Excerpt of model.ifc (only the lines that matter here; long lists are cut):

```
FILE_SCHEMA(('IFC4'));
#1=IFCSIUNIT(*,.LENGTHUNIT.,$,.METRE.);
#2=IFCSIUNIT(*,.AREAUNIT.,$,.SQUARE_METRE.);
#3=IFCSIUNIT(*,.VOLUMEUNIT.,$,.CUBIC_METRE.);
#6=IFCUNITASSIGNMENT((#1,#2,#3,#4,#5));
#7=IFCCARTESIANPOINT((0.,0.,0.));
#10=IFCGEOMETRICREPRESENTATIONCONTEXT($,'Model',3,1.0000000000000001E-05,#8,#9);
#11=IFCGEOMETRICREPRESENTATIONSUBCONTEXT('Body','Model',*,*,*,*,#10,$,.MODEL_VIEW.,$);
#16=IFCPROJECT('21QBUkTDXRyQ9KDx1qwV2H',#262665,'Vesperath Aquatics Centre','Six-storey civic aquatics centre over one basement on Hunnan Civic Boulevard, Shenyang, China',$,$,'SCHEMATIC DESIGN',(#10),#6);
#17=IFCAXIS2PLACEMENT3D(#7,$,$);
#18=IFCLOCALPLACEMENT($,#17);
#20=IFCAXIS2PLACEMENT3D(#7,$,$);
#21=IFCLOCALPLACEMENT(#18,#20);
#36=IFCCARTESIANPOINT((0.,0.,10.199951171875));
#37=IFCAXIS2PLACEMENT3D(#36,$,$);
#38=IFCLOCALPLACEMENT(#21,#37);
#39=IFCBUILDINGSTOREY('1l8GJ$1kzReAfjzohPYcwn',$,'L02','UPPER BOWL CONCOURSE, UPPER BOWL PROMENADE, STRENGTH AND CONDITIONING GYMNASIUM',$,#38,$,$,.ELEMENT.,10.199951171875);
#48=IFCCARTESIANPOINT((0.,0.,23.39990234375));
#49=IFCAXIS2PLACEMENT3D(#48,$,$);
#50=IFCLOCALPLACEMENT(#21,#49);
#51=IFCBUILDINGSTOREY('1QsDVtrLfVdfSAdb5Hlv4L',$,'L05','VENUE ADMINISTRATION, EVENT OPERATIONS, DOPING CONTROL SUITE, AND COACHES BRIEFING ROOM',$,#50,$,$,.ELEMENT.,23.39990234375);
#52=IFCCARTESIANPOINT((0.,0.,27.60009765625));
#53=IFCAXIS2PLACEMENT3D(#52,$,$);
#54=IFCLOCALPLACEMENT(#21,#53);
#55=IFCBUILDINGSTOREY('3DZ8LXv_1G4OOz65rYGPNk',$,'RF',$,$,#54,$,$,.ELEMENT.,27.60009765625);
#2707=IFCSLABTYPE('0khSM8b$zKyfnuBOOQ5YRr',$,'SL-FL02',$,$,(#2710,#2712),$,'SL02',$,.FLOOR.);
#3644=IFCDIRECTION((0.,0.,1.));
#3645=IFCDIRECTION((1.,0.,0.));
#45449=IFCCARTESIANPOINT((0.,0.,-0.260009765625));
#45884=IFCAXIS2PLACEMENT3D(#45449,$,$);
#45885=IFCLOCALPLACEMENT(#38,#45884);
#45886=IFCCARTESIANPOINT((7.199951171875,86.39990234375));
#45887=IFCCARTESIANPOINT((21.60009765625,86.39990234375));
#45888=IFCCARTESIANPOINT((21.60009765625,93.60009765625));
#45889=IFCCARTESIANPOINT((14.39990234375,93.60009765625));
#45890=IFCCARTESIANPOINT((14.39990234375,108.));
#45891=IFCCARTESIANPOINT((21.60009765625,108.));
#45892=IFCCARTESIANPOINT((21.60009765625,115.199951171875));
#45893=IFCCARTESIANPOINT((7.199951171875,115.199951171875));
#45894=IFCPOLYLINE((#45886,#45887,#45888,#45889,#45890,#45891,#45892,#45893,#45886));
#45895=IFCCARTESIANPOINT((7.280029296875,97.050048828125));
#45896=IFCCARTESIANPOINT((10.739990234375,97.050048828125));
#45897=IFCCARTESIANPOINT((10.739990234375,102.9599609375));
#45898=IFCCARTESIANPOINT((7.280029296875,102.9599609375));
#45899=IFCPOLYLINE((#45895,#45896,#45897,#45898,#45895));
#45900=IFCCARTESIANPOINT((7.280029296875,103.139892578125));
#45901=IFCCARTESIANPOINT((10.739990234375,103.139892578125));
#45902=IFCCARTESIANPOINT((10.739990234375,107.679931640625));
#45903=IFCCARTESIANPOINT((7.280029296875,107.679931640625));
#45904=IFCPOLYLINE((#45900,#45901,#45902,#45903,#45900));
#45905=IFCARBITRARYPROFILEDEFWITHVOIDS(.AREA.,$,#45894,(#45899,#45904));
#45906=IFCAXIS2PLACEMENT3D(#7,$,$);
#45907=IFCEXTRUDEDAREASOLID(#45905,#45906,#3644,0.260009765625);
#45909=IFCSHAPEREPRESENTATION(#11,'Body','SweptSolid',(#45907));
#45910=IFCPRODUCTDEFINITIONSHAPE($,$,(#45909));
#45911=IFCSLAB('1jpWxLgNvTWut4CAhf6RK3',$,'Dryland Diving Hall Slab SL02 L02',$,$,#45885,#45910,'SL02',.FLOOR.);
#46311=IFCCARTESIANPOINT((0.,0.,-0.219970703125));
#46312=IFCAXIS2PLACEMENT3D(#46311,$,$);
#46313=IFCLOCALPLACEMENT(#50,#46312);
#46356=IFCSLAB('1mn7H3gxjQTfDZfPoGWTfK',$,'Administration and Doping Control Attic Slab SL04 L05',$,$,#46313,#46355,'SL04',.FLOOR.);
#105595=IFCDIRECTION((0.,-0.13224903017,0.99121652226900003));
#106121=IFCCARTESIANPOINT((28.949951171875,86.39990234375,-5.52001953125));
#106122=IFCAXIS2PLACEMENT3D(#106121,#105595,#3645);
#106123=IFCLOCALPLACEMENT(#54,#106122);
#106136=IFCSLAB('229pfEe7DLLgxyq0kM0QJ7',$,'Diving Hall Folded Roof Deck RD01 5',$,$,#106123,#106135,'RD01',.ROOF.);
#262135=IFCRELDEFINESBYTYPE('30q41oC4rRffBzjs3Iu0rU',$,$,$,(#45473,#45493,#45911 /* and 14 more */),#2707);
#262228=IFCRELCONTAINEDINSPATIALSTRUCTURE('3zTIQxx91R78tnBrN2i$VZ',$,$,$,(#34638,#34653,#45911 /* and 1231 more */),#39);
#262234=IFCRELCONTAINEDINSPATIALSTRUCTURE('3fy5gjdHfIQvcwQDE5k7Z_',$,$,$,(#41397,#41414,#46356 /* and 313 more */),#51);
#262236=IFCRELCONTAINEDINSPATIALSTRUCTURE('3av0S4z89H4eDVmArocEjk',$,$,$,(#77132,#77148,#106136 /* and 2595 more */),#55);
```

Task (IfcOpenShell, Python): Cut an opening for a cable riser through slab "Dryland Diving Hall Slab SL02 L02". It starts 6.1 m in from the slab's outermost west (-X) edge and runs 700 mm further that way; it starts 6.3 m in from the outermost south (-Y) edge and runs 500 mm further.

```python
import numpy as np
import ifcopenshell
import ifcopenshell.api.feature
import ifcopenshell.api.geometry
import ifcopenshell.api.root
import ifcopenshell.geom
import ifcopenshell.util.placement
import ifcopenshell.util.representation
import ifcopenshell.util.shape
import ifcopenshell.util.unit

model = ifcopenshell.open("model.ifc")
unit_scale = ifcopenshell.util.unit.calculate_unit_scale(model)
settings = ifcopenshell.geom.settings()


def volume(element):
    """Net volume in cubic metres, openings subtracted."""
    shape = ifcopenshell.geom.create_shape(settings, element)
    return ifcopenshell.util.shape.get_volume(shape.geometry)


slab = model.by_id(45911)
before = volume(slab)

# Extent in the slab's own axes, in metres. The edges named are its -X and -Y sides.
slab_shape = ifcopenshell.geom.create_shape(settings, slab)
vertices = ifcopenshell.util.shape.get_vertices(slab_shape.geometry)
x_min, y_min, bottom = vertices.min(axis=0)
top = vertices[:, 2].max()

opening = ifcopenshell.api.root.create_entity(model, ifc_class="IfcOpeningElement", name="Cable riser opening", predefined_type="OPENING")
context = ifcopenshell.util.representation.get_context(model, "Model", "Body", "MODEL_VIEW")
width, depth = 0.7, 0.5
outline = [(0.0, 0.0), (width, 0.0), (width, depth), (0.0, depth), (0.0, 0.0)]
# Overshoot both faces by 50 mm so the cut is clean.
shape = ifcopenshell.api.geometry.add_slab_representation(
    model, context=context, depth=top - bottom + 0.1, polyline=outline
)
ifcopenshell.api.geometry.assign_representation(model, product=opening, representation=shape)

matrix = ifcopenshell.util.placement.get_local_placement(slab.ObjectPlacement)
matrix[:, 3] = matrix @ np.append(np.array([x_min + 6.1, y_min + 6.3, bottom - 0.05]) / unit_scale, 1.0)
ifcopenshell.api.geometry.edit_object_placement(model, product=opening, matrix=matrix, is_si=False)
ifcopenshell.api.feature.add_feature(model, feature=opening, element=slab)

after = volume(slab)

print(f"slab volume {before:.3f} -> {after:.3f} m3")

model.write("model_rev.ifc")
```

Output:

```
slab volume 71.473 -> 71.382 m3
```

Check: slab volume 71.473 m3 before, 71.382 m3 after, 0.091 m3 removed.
